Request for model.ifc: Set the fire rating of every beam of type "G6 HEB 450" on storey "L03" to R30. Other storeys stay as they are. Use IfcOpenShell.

First a look at what the model holds.

```python
import ifcopenshell
import ifcopenshell.util.element

model = ifcopenshell.open("model.ifc")
print(model.schema)
storey = next(s for s in model.by_type("IfcBuildingStorey") if s.Name == "L03")
beams = [e for e in ifcopenshell.util.element.get_decomposition(storey) if e.is_a("IfcBeam")]
seen = {}
for e in beams:
    element_type = ifcopenshell.util.element.get_type(e)
    key = (element_type.Name if element_type != e and element_type else None, ifcopenshell.util.element.get_pset(e, "Pset_BeamCommon", "FireRating"))
    seen[key] = seen.get(key, 0) + 1
for (name, value), count in sorted(seen.items(), key=str):
    print(count, "x", name, "|", value)
```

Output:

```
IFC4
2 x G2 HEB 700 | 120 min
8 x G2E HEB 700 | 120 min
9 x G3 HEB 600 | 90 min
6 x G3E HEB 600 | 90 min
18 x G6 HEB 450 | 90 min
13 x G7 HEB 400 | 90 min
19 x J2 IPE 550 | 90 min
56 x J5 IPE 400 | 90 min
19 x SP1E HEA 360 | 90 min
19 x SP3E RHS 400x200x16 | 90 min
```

```python
import ifcopenshell
import ifcopenshell.api.pset
import ifcopenshell.util.element

model = ifcopenshell.open("model.ifc")

storey = next(s for s in model.by_type("IfcBuildingStorey") if s.Name == "L03")
beams = [e for e in ifcopenshell.util.element.get_decomposition(storey) if e.is_a("IfcBeam")]

count = 0
for e in beams:
    element_type = ifcopenshell.util.element.get_type(e)
    if element_type in (None, e) or element_type.Name != "G6 HEB 450":
        continue
    # add_pset returns the element's existing set when there is one.
    pset = ifcopenshell.api.pset.add_pset(model, product=e, name="Pset_BeamCommon")
    ifcopenshell.api.pset.edit_pset(model, pset=pset, properties={"FireRating": "R30"})
    count += 1

print(count, "beams updated")

model.write("model_rev.ifc")
```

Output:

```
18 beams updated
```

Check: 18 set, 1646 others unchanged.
